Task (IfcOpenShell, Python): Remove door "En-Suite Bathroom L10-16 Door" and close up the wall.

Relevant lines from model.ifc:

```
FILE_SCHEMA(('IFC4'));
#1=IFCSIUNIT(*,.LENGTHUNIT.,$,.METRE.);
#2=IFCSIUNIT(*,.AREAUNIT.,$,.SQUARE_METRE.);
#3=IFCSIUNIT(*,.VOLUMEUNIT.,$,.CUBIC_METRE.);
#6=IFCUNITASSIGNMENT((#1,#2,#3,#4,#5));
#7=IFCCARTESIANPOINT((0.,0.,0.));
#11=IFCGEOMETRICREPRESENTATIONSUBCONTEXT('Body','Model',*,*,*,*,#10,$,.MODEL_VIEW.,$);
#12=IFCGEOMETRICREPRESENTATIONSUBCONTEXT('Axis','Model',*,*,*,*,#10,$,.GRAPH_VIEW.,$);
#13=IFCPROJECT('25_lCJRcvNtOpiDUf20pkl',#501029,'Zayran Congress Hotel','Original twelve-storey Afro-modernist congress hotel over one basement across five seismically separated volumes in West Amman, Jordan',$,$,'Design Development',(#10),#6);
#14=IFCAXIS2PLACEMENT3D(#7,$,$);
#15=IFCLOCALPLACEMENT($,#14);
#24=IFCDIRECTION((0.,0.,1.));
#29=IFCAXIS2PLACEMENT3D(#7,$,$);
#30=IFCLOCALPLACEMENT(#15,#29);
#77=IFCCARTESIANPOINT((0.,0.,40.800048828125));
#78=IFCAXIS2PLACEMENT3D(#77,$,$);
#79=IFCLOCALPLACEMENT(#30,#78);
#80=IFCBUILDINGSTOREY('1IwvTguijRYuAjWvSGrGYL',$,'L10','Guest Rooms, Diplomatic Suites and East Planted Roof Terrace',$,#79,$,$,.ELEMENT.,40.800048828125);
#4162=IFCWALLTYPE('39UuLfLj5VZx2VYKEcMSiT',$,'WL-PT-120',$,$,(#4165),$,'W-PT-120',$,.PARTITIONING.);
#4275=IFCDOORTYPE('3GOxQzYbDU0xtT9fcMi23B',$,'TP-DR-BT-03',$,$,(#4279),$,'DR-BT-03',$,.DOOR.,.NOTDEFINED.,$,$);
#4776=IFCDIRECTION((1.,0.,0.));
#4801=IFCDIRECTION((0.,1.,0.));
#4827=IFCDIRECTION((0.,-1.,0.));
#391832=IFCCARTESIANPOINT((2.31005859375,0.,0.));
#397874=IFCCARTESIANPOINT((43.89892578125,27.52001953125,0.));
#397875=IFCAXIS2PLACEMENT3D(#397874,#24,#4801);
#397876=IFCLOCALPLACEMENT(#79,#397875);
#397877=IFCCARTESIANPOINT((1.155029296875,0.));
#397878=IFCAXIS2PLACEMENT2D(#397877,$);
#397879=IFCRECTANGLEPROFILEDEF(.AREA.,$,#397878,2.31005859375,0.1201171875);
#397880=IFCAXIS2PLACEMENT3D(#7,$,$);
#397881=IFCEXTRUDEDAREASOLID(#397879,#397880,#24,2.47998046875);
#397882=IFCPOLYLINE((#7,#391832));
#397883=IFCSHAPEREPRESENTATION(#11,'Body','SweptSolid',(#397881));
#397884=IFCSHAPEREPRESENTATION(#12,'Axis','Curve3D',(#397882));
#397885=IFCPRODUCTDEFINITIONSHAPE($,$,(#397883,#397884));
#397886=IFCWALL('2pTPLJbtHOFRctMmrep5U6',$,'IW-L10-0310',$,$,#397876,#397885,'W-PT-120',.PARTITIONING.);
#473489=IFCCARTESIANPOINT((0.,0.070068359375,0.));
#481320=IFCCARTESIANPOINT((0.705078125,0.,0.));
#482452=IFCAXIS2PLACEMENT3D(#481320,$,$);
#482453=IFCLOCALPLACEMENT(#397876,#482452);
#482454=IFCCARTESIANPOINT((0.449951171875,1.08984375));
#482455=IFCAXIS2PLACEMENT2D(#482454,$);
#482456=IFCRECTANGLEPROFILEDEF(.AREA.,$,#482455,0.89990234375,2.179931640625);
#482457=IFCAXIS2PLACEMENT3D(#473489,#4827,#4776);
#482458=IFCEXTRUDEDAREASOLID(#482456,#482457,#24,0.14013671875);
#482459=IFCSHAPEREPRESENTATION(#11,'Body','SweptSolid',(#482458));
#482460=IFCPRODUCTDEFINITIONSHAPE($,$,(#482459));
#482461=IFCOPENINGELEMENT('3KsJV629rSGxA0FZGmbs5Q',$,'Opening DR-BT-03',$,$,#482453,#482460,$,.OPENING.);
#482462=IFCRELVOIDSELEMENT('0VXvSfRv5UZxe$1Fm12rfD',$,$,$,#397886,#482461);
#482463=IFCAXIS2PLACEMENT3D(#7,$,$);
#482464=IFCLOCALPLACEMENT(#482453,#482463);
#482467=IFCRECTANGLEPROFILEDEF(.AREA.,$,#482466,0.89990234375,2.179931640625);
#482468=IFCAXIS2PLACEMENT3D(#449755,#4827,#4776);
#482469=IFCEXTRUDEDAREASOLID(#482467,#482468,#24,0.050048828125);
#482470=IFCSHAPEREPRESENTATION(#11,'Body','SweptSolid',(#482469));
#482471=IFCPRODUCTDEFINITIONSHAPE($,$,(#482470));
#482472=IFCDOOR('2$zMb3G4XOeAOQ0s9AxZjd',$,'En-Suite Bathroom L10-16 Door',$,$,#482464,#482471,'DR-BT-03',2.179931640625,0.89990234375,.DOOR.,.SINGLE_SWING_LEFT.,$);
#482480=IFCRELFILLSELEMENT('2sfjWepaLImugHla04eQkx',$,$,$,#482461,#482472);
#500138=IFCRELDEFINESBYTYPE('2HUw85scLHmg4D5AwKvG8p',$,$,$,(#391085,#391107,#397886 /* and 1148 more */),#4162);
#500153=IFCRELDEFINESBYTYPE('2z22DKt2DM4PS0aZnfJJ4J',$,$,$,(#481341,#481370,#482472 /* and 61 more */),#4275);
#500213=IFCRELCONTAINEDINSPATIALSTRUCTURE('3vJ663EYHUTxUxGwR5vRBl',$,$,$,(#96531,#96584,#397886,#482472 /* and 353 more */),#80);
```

```python
import ifcopenshell
import ifcopenshell.api.feature
import ifcopenshell.api.root
import ifcopenshell.geom
import ifcopenshell.util.shape

model = ifcopenshell.open("model.ifc")
settings = ifcopenshell.geom.settings()


def volume(element):
    """Net volume in cubic metres, openings subtracted."""
    shape = ifcopenshell.geom.create_shape(settings, element)
    return ifcopenshell.util.shape.get_volume(shape.geometry)


door = model.by_guid("2$zMb3G4XOeAOQ0s9AxZjd")
opening = door.FillsVoids[0].RelatingOpeningElement
wall = opening.VoidsElements[0].RelatingBuildingElement
before = volume(wall)

ifcopenshell.api.root.remove_product(model, product=door)
ifcopenshell.api.feature.remove_feature(model, feature=opening)

after = volume(wall)

print(f"wall volume {before:.3f} -> {after:.3f} m3")

model.write("model_v2.ifc")
```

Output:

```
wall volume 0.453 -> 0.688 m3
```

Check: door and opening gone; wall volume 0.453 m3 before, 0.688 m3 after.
